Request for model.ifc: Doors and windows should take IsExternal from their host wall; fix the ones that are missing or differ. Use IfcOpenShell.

First a look at what the model holds.

```python
import ifcopenshell
import ifcopenshell.util.element

model = ifcopenshell.open("model.ifc")
print(model.schema)
seen = {}
for e in model.by_type("IfcDoor") + model.by_type("IfcWindow"):
    if not e.FillsVoids:
        continue
    host = e.FillsVoids[0].RelatingOpeningElement.VoidsElements[0].RelatingBuildingElement
    own = ifcopenshell.util.element.get_pset(e, f"Pset_{e.is_a()[3:].removesuffix('StandardCase')}Common", "IsExternal")
    wall = ifcopenshell.util.element.get_pset(host, "Pset_WallCommon", "IsExternal")
    seen[e.is_a(), own, wall] = seen.get((e.is_a(), own, wall), 0) + 1
for (cls, own, wall), count in sorted(seen.items(), key=str):
    print(count, cls, "IsExternal:", own, "| host wall:", wall)
```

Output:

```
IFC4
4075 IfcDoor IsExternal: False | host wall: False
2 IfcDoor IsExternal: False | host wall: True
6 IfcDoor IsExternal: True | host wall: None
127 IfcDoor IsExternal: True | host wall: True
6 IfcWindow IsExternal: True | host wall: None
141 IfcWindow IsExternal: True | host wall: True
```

```python
import ifcopenshell
import ifcopenshell.api.pset
import ifcopenshell.util.element

model = ifcopenshell.open("model.ifc")

count = 0
for ifc_class, pset_name in (("IfcDoor", "Pset_DoorCommon"), ("IfcWindow", "Pset_WindowCommon")):
    for e in model.by_type(ifc_class):
        if not e.FillsVoids:
            continue
        host = e.FillsVoids[0].RelatingOpeningElement.VoidsElements[0].RelatingBuildingElement
        external = ifcopenshell.util.element.get_pset(host, "Pset_WallCommon", "IsExternal")
        if external is None or ifcopenshell.util.element.get_pset(e, pset_name, "IsExternal") == external:
            continue
        pset = ifcopenshell.api.pset.add_pset(model, product=e, name=pset_name)
        ifcopenshell.api.pset.edit_pset(model, pset=pset, properties={"IsExternal": external})
        count += 1

print(count, "updated")

model.write("model_updated.ifc")
```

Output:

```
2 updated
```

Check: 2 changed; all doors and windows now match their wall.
